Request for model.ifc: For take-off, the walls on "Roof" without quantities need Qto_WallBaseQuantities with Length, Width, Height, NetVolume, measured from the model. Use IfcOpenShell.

First a look at what the model holds.

```python
import ifcopenshell
import ifcopenshell.util.element
import ifcopenshell.util.unit

model = ifcopenshell.open("model.ifc")
print(model.schema)
for unit_type in ("LENGTHUNIT", "AREAUNIT", "VOLUMEUNIT"):
    print(unit_type, ifcopenshell.util.unit.calculate_unit_scale(model, unit_type))
storey = next(s for s in model.by_type("IfcBuildingStorey") if s.Name == "Roof")
walls = [e for e in ifcopenshell.util.element.get_decomposition(storey) if e.is_a("IfcWall")]
for e in sorted(walls, key=lambda e: e.id()):
    print(e.id(), e.is_a(), e.Name, list(ifcopenshell.util.element.get_psets(e, qtos_only=True)), sep=" | ")
```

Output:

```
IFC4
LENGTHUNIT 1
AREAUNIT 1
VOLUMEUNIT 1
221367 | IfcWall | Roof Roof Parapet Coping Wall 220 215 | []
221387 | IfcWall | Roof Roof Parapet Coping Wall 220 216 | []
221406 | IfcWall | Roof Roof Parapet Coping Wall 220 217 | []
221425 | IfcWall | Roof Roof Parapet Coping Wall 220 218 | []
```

```python
import ifcopenshell
import ifcopenshell.api.pset
import ifcopenshell.geom
import ifcopenshell.util.element
import ifcopenshell.util.shape
import ifcopenshell.util.unit

model = ifcopenshell.open("model.ifc")
unit_scale = ifcopenshell.util.unit.calculate_unit_scale(model)
volume_scale = ifcopenshell.util.unit.calculate_unit_scale(model, "VOLUMEUNIT")
settings = ifcopenshell.geom.settings()

storey = next(s for s in model.by_type("IfcBuildingStorey") if s.Name == "Roof")
walls = [e for e in ifcopenshell.util.element.get_decomposition(storey) if e.is_a("IfcWall")]

for e in sorted(walls, key=lambda e: e.id()):
    if ifcopenshell.util.element.get_psets(e, qtos_only=True, should_inherit=False):
        continue
    # Geometry comes back in metres, in the element's own axes.
    shape = ifcopenshell.geom.create_shape(settings, e)
    values = {
        "Length": ifcopenshell.util.shape.get_x(shape.geometry) / unit_scale,
        "Width": ifcopenshell.util.shape.get_y(shape.geometry) / unit_scale,
        "Height": ifcopenshell.util.shape.get_z(shape.geometry) / unit_scale,
        "NetVolume": ifcopenshell.util.shape.get_volume(shape.geometry) / volume_scale,
    }
    qto = ifcopenshell.api.pset.add_qto(model, product=e, name="Qto_WallBaseQuantities")
    ifcopenshell.api.pset.edit_qto(model, qto=qto, properties=values)
    print(e.id(), {k: round(v, 3) for k, v in values.items()})

model.write("model-out.ifc")
```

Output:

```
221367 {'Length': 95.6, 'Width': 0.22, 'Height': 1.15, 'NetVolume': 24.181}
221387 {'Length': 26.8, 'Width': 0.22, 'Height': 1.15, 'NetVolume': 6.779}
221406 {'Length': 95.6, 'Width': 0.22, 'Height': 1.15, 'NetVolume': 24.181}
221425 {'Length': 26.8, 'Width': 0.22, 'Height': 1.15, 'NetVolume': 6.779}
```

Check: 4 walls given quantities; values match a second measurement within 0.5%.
